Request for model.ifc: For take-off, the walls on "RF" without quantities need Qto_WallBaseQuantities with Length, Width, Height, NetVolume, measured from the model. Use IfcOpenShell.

First a look at what the model holds.

```python
import ifcopenshell
import ifcopenshell.util.element
import ifcopenshell.util.unit

model = ifcopenshell.open("model.ifc")
print(model.schema)
for unit_type in ("LENGTHUNIT", "AREAUNIT", "VOLUMEUNIT"):
    print(unit_type, ifcopenshell.util.unit.calculate_unit_scale(model, unit_type))
storey = next(s for s in model.by_type("IfcBuildingStorey") if s.Name == "RF")
walls = [e for e in ifcopenshell.util.element.get_decomposition(storey) if e.is_a("IfcWall")]
for e in sorted(walls, key=lambda e: e.id()):
    print(e.id(), e.is_a(), e.Name, list(ifcopenshell.util.element.get_psets(e, qtos_only=True)), sep=" | ")
```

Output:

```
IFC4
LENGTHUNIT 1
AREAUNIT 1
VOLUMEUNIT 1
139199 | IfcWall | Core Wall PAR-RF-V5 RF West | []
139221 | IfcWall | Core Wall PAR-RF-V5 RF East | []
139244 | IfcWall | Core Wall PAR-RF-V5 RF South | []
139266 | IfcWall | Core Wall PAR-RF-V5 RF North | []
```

```python
import ifcopenshell
import ifcopenshell.api.pset
import ifcopenshell.geom
import ifcopenshell.util.element
import ifcopenshell.util.shape
import ifcopenshell.util.unit

model = ifcopenshell.open("model.ifc")
unit_scale = ifcopenshell.util.unit.calculate_unit_scale(model)
volume_scale = ifcopenshell.util.unit.calculate_unit_scale(model, "VOLUMEUNIT")
settings = ifcopenshell.geom.settings()

storey = next(s for s in model.by_type("IfcBuildingStorey") if s.Name == "RF")
walls = [e for e in ifcopenshell.util.element.get_decomposition(storey) if e.is_a("IfcWall")]

for e in sorted(walls, key=lambda e: e.id()):
    if ifcopenshell.util.element.get_psets(e, qtos_only=True, should_inherit=False):
        continue
    # Geometry comes back in metres, in the element's own axes.
    shape = ifcopenshell.geom.create_shape(settings, e)
    values = {
        "Length": ifcopenshell.util.shape.get_x(shape.geometry) / unit_scale,
        "Width": ifcopenshell.util.shape.get_y(shape.geometry) / unit_scale,
        "Height": ifcopenshell.util.shape.get_z(shape.geometry) / unit_scale,
        "NetVolume": ifcopenshell.util.shape.get_volume(shape.geometry) / volume_scale,
    }
    qto = ifcopenshell.api.pset.add_qto(model, product=e, name="Qto_WallBaseQuantities")
    ifcopenshell.api.pset.edit_qto(model, qto=qto, properties=values)
    print(e.id(), {k: round(v, 3) for k, v in values.items()})

model.write("model_rev.ifc")
```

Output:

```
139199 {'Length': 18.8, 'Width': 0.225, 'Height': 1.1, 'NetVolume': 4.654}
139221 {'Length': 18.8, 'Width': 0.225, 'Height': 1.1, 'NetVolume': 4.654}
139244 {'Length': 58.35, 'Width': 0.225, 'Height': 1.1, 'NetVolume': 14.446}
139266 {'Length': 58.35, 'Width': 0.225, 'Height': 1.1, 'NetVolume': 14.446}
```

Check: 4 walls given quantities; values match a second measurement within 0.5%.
